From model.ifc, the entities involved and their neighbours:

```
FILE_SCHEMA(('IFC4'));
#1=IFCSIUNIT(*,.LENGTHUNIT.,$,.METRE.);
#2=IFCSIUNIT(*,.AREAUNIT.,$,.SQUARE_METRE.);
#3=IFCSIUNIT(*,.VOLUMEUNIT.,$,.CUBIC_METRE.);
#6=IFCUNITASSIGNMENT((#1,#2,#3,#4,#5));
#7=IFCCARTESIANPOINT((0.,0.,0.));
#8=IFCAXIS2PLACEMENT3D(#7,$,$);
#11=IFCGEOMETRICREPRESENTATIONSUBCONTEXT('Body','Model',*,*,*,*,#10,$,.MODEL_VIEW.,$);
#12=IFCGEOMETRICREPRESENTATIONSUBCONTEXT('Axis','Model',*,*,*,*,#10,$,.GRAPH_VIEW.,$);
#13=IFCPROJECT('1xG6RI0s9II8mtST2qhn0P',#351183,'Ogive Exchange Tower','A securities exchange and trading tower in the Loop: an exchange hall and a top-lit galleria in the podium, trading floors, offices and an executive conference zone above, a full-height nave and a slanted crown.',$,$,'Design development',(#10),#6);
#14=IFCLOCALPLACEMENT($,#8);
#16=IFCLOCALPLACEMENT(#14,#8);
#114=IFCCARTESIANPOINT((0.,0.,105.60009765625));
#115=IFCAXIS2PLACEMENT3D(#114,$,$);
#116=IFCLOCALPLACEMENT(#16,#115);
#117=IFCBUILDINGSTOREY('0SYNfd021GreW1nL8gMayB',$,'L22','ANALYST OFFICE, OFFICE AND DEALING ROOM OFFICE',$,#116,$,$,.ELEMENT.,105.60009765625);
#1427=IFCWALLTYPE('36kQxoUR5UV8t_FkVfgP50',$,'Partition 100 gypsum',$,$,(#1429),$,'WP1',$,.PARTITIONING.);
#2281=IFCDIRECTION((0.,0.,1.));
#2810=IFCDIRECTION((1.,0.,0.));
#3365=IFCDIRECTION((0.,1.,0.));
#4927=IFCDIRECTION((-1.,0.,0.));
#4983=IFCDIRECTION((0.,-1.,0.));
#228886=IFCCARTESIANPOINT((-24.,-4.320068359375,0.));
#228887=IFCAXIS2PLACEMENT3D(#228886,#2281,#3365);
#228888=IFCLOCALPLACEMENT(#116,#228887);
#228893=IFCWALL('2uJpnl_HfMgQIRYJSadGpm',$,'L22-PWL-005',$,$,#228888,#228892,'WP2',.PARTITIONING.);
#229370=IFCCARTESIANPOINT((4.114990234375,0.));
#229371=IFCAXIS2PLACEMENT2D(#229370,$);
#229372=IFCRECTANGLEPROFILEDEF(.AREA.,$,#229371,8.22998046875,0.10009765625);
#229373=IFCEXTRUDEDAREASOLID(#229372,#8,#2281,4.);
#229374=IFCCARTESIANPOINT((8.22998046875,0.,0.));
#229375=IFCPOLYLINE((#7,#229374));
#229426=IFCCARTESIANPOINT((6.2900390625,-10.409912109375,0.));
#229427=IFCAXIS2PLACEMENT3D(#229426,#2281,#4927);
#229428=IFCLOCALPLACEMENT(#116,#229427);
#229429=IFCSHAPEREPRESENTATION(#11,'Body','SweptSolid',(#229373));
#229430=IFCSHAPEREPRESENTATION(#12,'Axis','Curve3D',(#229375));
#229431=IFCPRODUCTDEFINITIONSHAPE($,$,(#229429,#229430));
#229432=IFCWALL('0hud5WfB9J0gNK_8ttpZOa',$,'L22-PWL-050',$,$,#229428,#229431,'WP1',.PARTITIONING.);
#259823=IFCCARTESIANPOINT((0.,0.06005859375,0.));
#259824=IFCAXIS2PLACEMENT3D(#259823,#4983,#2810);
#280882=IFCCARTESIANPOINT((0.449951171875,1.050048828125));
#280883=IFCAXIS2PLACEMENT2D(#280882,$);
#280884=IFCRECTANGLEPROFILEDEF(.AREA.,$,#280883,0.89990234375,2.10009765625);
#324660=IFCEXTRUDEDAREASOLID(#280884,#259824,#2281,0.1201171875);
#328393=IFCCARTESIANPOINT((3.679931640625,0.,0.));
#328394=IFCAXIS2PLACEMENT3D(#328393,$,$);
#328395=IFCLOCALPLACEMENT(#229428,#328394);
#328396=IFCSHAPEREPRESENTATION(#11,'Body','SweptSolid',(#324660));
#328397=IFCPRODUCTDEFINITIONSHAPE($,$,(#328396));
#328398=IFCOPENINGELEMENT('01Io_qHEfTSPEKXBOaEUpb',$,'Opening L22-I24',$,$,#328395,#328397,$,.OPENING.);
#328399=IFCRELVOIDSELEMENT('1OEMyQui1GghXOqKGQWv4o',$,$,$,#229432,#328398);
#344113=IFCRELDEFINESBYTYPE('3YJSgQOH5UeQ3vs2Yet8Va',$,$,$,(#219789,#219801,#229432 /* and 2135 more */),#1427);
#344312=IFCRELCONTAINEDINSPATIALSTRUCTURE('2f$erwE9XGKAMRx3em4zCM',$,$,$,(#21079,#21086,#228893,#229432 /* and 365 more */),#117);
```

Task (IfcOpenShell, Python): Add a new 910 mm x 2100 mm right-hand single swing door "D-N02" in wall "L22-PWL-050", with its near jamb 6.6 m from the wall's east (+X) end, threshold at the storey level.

```python
import numpy as np
import ifcopenshell
import ifcopenshell.api.feature
import ifcopenshell.api.geometry
import ifcopenshell.api.root
import ifcopenshell.api.spatial
import ifcopenshell.geom
import ifcopenshell.util.element
import ifcopenshell.util.placement
import ifcopenshell.util.representation
import ifcopenshell.util.shape
import ifcopenshell.util.unit

model = ifcopenshell.open("model.ifc")
unit_scale = ifcopenshell.util.unit.calculate_unit_scale(model)
settings = ifcopenshell.geom.settings()


def volume(element):
    """Net volume in cubic metres, openings subtracted."""
    shape = ifcopenshell.geom.create_shape(settings, element)
    return ifcopenshell.util.shape.get_volume(shape.geometry)


wall = model.by_guid("0hud5WfB9J0gNK_8ttpZOa")
storey = ifcopenshell.util.element.get_container(wall, ifc_class="IfcBuildingStorey")
context = ifcopenshell.util.representation.get_context(model, "Model", "Body", "MODEL_VIEW")
before = volume(wall)

width, height, from_end, sill = 0.91, 2.1, 6.6, 0.0  # metres

# The wall runs along its own X axis, and the end named is its -X end.
wall_shape = ifcopenshell.geom.create_shape(settings, wall)
x, y, z = ifcopenshell.util.shape.get_vertices(wall_shape.geometry).T
start = x.min() + from_end
face, thickness = float(y.min()), float(y.max() - y.min())
wall_matrix = ifcopenshell.util.placement.get_local_placement(wall.ObjectPlacement)
level = ifcopenshell.util.placement.get_local_placement(storey.ObjectPlacement)[2, 3]


def in_wall(x, y):
    """Placement at x, y metres in the wall's axes, at sill height."""
    matrix = wall_matrix.copy()
    matrix[:, 3] = wall_matrix @ np.array([x / unit_scale, y / unit_scale, 0.0, 1.0])
    matrix[2, 3] = level + sill / unit_scale
    return matrix


# Opening: a box that overshoots both wall faces by 50 mm.
opening = ifcopenshell.api.root.create_entity(model, ifc_class="IfcOpeningElement", predefined_type="OPENING")
box = ifcopenshell.api.geometry.add_wall_representation(
    model, context=context, length=width, height=height, thickness=thickness + 0.1
)
ifcopenshell.api.geometry.assign_representation(model, product=opening, representation=box)
ifcopenshell.api.geometry.edit_object_placement(model, product=opening, matrix=in_wall(start, face - 0.05), is_si=False)
ifcopenshell.api.feature.add_feature(model, feature=opening, element=wall)

door = ifcopenshell.api.root.create_entity(model, ifc_class="IfcDoor", name="D-N02", predefined_type="DOOR")
door.OverallWidth, door.OverallHeight = width / unit_scale, height / unit_scale
door.OperationType = "SINGLE_SWING_RIGHT"
body = ifcopenshell.api.geometry.add_door_representation(
    model,
    context=context,
    overall_width=door.OverallWidth,
    overall_height=door.OverallHeight,
    operation_type="SINGLE_SWING_RIGHT",
    lining_properties={"LiningDepth": thickness / unit_scale, "ThresholdDepth": thickness / unit_scale},
)
ifcopenshell.api.geometry.assign_representation(model, product=door, representation=body)
ifcopenshell.api.spatial.assign_container(model, products=[door], relating_structure=storey)
ifcopenshell.api.feature.add_filling(model, opening=opening, element=door)

# The lining spans the wall, so the door starts at the wall face.
ifcopenshell.api.geometry.edit_object_placement(model, product=door, matrix=in_wall(start, face), is_si=False)

after = volume(wall)

print(f"wall volume {before:.3f} -> {after:.3f} m3")

model.write("model_v2.ifc")
```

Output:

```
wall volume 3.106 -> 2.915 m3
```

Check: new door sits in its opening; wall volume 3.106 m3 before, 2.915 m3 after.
